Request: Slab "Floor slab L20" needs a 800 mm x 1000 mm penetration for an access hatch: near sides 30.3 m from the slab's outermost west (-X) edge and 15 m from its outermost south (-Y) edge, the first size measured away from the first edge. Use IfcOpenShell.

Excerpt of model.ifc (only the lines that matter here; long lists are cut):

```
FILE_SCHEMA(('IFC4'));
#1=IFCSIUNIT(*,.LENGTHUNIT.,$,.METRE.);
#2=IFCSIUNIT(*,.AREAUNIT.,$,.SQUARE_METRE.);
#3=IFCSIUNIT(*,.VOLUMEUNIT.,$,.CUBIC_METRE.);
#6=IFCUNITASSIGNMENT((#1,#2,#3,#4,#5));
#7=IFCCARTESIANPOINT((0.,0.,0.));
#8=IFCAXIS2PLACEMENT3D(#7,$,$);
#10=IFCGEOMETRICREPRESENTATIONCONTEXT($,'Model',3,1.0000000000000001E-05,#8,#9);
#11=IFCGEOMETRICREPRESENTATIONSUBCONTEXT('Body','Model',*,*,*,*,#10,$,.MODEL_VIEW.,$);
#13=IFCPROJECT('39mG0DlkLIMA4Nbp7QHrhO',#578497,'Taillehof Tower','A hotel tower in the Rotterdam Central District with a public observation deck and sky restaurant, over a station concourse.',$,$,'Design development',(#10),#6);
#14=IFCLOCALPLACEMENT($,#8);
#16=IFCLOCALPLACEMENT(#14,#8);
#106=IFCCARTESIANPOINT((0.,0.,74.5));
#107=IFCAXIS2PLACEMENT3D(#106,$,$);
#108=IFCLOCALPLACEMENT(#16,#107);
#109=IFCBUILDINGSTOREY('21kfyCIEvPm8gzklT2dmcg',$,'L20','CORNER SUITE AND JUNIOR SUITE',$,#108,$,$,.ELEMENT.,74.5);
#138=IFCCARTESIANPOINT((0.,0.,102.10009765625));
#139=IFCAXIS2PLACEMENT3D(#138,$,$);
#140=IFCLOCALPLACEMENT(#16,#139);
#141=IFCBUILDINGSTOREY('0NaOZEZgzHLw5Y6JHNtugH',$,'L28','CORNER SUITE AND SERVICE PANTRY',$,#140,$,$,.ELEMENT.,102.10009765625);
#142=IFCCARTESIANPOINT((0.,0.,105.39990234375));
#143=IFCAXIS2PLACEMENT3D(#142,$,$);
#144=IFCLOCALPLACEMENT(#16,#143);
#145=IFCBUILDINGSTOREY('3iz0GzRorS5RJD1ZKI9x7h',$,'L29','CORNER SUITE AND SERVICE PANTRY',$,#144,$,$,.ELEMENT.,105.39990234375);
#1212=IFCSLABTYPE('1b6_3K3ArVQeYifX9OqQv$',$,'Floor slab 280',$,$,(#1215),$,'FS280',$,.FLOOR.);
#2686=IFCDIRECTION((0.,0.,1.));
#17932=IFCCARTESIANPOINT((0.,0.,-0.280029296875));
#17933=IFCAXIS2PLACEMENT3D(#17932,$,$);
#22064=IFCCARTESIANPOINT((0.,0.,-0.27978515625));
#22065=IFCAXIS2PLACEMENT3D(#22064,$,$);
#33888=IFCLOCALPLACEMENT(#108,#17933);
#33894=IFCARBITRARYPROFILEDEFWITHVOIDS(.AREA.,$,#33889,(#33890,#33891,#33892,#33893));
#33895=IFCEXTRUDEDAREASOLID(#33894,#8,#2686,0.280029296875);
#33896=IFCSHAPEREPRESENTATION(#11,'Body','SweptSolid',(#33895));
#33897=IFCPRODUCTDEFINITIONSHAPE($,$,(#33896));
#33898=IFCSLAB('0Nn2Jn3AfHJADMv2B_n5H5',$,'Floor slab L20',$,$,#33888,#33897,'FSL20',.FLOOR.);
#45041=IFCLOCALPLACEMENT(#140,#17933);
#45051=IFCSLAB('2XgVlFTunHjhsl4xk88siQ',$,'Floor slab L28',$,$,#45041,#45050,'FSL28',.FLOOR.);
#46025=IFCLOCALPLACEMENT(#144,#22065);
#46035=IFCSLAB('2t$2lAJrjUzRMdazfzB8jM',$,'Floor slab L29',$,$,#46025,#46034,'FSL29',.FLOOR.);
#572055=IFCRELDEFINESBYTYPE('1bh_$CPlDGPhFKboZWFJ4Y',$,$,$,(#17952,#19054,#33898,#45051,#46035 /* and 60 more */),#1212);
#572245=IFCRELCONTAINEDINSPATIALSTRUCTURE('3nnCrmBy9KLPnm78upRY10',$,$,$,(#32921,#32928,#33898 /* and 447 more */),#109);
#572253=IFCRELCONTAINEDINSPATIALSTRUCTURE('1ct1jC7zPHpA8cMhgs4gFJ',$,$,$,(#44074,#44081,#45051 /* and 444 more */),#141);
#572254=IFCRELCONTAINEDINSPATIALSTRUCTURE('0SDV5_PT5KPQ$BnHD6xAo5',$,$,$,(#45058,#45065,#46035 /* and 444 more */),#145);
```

```python
import numpy as np
import ifcopenshell
import ifcopenshell.api.feature
import ifcopenshell.api.geometry
import ifcopenshell.api.root
import ifcopenshell.geom
import ifcopenshell.util.placement
import ifcopenshell.util.representation
import ifcopenshell.util.shape
import ifcopenshell.util.unit

model = ifcopenshell.open("model.ifc")
unit_scale = ifcopenshell.util.unit.calculate_unit_scale(model)
settings = ifcopenshell.geom.settings()


def volume(element):
    """Net volume in cubic metres, openings subtracted."""
    shape = ifcopenshell.geom.create_shape(settings, element)
    return ifcopenshell.util.shape.get_volume(shape.geometry)


slab = model.by_guid("0Nn2Jn3AfHJADMv2B_n5H5")
before = volume(slab)

# Extent in the slab's own axes, in metres. The edges named are its -X and -Y sides.
slab_shape = ifcopenshell.geom.create_shape(settings, slab)
vertices = ifcopenshell.util.shape.get_vertices(slab_shape.geometry)
x_min, y_min, bottom = vertices.min(axis=0)
top = vertices[:, 2].max()

opening = ifcopenshell.api.root.create_entity(model, ifc_class="IfcOpeningElement", name="Access hatch opening", predefined_type="OPENING")
context = ifcopenshell.util.representation.get_context(model, "Model", "Body", "MODEL_VIEW")
width, depth = 0.8, 1
outline = [(0.0, 0.0), (width, 0.0), (width, depth), (0.0, depth), (0.0, 0.0)]
# Overshoot both faces by 50 mm so the cut is clean.
shape = ifcopenshell.api.geometry.add_slab_representation(
    model, context=context, depth=top - bottom + 0.1, polyline=outline
)
ifcopenshell.api.geometry.assign_representation(model, product=opening, representation=shape)

matrix = ifcopenshell.util.placement.get_local_placement(slab.ObjectPlacement)
matrix[:, 3] = matrix @ np.append(np.array([x_min + 30.3, y_min + 15, bottom - 0.05]) / unit_scale, 1.0)
ifcopenshell.api.geometry.edit_object_placement(model, product=opening, matrix=matrix, is_si=False)
ifcopenshell.api.feature.add_feature(model, feature=opening, element=slab)

after = volume(slab)

print(f"slab volume {before:.3f} -> {after:.3f} m3")

model.write("model_edited.ifc")
```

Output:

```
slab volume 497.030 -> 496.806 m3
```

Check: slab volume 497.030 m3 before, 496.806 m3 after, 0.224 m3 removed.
